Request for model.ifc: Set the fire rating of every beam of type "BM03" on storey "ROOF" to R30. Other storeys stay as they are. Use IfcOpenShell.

First a look at what the model holds.

```python
import ifcopenshell
import ifcopenshell.util.element

model = ifcopenshell.open("model.ifc")
print(model.schema)
storey = next(s for s in model.by_type("IfcBuildingStorey") if s.Name == "ROOF")
beams = [e for e in ifcopenshell.util.element.get_decomposition(storey) if e.is_a("IfcBeam")]
seen = {}
for e in beams:
    element_type = ifcopenshell.util.element.get_type(e)
    key = (element_type.Name if element_type != e and element_type else None, ifcopenshell.util.element.get_pset(e, "Pset_BeamCommon", "FireRating"))
    seen[key] = seen.get(key, 0) + 1
for (name, value), count in sorted(seen.items(), key=str):
    print(count, "x", name, "|", value)
```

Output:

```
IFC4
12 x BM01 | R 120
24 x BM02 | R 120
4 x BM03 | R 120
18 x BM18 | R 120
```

```python
import ifcopenshell
import ifcopenshell.api.pset
import ifcopenshell.util.element

model = ifcopenshell.open("model.ifc")

storey = next(s for s in model.by_type("IfcBuildingStorey") if s.Name == "ROOF")
beams = [e for e in ifcopenshell.util.element.get_decomposition(storey) if e.is_a("IfcBeam")]

count = 0
for e in beams:
    element_type = ifcopenshell.util.element.get_type(e)
    if element_type in (None, e) or element_type.Name != "BM03":
        continue
    # add_pset returns the element's existing set when there is one.
    pset = ifcopenshell.api.pset.add_pset(model, product=e, name="Pset_BeamCommon")
    ifcopenshell.api.pset.edit_pset(model, pset=pset, properties={"FireRating": "R30"})
    count += 1

print(count, "beams updated")

model.write("model_rev.ifc")
```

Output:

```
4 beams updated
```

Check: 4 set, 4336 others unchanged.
